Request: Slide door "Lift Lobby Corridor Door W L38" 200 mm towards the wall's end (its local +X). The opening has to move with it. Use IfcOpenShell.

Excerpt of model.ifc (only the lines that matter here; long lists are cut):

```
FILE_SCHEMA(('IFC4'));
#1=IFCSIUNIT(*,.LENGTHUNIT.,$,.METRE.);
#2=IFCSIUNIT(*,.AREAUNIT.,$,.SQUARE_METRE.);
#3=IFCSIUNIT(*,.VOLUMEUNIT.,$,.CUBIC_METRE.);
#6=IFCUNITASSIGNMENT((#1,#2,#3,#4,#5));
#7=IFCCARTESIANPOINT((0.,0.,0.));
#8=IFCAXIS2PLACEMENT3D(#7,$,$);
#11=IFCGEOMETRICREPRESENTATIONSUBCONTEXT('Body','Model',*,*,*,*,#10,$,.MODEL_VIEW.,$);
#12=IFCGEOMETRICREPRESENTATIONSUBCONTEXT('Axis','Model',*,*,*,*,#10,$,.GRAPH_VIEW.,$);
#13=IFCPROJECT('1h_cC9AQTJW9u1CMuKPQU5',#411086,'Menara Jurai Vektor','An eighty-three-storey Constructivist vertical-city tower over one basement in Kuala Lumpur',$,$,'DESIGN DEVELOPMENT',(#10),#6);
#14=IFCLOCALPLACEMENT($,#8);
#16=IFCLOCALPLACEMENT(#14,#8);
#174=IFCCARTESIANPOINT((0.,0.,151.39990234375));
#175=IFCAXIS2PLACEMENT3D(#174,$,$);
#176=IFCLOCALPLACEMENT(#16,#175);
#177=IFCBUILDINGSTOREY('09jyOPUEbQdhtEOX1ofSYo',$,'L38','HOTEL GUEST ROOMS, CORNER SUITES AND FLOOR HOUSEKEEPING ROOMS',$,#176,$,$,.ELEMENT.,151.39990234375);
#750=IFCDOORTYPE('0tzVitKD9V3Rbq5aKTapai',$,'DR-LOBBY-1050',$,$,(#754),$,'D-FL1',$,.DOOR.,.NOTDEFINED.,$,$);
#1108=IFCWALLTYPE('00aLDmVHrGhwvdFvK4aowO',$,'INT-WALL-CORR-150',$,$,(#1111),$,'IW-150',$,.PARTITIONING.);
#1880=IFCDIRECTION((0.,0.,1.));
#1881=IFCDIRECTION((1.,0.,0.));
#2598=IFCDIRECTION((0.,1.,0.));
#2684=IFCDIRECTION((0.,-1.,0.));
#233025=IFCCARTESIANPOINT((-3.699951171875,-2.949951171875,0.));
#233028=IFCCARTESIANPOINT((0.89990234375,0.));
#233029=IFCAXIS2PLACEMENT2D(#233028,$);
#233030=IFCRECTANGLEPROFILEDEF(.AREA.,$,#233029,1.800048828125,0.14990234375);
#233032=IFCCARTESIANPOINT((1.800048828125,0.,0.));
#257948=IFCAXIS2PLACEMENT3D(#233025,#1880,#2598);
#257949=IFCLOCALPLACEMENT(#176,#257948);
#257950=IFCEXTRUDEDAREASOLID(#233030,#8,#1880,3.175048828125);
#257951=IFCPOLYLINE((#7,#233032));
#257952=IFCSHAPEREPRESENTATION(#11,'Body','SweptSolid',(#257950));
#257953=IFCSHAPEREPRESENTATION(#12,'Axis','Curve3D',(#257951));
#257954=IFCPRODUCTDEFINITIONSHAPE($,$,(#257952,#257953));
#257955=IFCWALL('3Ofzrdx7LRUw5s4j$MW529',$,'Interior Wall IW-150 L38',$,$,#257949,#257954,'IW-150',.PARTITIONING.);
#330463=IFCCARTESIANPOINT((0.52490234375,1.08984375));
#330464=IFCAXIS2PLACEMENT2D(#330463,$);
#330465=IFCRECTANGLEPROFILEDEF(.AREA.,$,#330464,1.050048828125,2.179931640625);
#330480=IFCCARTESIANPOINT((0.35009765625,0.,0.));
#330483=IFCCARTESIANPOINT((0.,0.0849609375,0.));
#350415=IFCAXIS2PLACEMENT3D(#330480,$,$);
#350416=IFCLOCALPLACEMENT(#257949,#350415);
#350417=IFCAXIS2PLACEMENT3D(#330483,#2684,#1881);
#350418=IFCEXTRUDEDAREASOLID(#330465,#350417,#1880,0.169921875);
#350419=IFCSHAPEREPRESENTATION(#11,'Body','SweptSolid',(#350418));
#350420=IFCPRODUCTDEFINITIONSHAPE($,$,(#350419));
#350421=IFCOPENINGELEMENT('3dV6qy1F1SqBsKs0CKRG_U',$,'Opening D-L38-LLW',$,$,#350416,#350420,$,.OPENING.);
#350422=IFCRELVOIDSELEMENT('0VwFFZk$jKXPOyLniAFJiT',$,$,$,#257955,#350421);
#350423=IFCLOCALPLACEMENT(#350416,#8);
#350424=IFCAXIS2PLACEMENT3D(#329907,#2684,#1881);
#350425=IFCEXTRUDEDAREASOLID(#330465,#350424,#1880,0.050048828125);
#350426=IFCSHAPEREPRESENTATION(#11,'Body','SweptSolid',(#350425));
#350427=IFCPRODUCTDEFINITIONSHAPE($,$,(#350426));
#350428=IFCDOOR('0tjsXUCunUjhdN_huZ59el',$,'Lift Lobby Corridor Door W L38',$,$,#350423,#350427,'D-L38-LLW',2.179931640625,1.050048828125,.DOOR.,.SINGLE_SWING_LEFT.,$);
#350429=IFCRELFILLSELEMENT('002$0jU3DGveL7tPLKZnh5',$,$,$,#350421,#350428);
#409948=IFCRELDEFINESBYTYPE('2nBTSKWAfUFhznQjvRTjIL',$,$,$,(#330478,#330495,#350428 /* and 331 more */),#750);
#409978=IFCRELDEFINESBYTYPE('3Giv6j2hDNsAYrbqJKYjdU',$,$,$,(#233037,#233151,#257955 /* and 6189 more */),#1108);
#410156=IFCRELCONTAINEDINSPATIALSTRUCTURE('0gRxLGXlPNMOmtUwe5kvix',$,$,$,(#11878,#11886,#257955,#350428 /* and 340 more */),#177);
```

```python
import ifcopenshell
import ifcopenshell.api.geometry
import ifcopenshell.util.placement
import ifcopenshell.util.unit

model = ifcopenshell.open("model.ifc")
unit_scale = ifcopenshell.util.unit.calculate_unit_scale(model)

door = model.by_guid("0tjsXUCunUjhdN_huZ59el")
opening = door.FillsVoids[0].RelatingOpeningElement
wall = opening.VoidsElements[0].RelatingBuildingElement

wall_matrix = ifcopenshell.util.placement.get_local_placement(wall.ObjectPlacement)
shift = wall_matrix[:3, 0] * 0.2 / unit_scale
before = ifcopenshell.util.placement.get_local_placement(door.ObjectPlacement)[:3, 3].copy()

# The door is placed relative to its opening, so it follows when the opening moves.
matrix = ifcopenshell.util.placement.get_local_placement(opening.ObjectPlacement)
matrix[:3, 3] += shift
ifcopenshell.api.geometry.edit_object_placement(
    model, product=opening, matrix=matrix, is_si=False, should_transform_children=True
)

after = ifcopenshell.util.placement.get_local_placement(door.ObjectPlacement)[:3, 3]
print("door moved by", (after - before).round(3) + 0.0)

model.write("model-out.ifc")
```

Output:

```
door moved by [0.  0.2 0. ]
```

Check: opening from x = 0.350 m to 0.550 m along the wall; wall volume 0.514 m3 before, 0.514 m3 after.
